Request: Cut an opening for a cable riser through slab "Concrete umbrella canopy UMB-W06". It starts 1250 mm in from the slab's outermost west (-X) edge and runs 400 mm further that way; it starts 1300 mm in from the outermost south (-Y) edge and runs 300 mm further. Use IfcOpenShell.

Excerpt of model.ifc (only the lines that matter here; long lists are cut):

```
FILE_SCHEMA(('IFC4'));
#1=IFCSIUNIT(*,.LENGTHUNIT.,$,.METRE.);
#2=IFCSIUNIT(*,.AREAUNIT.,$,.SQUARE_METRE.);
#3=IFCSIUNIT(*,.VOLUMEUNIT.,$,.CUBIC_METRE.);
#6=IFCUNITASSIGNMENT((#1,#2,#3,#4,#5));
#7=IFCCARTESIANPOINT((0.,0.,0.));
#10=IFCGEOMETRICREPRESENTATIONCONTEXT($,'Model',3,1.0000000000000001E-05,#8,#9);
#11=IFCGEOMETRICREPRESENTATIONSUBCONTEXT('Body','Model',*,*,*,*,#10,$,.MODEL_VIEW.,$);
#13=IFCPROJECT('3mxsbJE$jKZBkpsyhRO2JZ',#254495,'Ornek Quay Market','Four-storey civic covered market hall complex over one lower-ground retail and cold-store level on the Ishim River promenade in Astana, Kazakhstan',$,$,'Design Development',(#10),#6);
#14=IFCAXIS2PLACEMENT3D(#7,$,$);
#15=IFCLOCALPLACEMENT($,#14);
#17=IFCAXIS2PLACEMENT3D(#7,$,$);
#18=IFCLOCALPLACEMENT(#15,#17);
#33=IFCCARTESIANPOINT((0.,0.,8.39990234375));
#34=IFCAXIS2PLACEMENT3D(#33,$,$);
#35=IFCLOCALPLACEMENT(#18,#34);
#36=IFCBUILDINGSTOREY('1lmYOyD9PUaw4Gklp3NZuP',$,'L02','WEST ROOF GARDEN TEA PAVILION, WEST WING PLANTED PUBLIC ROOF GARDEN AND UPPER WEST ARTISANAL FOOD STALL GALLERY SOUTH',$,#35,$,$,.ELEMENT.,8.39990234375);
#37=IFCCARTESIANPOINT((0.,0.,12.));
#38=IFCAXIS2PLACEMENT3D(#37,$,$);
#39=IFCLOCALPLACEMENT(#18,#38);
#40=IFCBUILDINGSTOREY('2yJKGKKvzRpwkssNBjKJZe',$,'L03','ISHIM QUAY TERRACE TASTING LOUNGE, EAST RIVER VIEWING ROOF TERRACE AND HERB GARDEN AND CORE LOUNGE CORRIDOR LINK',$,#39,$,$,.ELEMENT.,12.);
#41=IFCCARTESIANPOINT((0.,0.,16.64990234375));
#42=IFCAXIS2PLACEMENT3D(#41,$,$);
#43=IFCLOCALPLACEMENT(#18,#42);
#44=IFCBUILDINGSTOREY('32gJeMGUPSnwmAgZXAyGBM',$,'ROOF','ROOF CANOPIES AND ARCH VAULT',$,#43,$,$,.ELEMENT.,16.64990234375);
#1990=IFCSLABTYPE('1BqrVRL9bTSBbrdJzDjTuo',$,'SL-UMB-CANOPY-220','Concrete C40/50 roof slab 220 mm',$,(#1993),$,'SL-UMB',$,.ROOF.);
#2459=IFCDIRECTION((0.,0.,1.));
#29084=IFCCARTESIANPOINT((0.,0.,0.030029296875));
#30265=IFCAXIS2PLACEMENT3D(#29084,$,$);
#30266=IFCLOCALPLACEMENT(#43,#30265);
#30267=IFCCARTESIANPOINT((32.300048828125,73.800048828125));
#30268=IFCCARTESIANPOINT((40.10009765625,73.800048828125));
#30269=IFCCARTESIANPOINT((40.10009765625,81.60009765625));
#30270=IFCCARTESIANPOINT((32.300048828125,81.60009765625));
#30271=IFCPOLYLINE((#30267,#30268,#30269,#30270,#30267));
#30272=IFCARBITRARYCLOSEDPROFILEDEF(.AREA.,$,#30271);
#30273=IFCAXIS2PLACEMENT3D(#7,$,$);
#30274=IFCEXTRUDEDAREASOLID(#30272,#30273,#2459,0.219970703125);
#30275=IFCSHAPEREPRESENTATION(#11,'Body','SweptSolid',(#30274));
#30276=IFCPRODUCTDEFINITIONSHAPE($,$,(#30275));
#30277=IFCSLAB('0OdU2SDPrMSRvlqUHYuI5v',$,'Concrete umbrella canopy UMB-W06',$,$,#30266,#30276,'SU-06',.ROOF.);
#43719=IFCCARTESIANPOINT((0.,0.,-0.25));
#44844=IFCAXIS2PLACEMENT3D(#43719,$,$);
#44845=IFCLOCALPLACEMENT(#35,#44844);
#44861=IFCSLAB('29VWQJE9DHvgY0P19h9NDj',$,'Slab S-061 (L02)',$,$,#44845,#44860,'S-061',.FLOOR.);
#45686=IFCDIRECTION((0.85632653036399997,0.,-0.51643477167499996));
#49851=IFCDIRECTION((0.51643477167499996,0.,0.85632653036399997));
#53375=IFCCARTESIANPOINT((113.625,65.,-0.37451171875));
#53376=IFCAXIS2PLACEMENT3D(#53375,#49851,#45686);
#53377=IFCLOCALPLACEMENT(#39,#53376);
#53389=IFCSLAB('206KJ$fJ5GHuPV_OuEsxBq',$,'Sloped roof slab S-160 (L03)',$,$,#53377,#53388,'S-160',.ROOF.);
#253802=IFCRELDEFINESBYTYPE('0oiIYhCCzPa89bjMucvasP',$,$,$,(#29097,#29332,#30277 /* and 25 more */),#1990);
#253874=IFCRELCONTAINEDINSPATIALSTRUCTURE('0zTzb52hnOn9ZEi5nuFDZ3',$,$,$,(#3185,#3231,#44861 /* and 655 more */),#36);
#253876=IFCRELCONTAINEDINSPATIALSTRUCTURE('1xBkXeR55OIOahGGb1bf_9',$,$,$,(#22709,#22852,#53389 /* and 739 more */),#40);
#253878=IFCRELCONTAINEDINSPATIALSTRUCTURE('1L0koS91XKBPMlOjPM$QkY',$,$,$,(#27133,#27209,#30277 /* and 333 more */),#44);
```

```python
import numpy as np
import ifcopenshell
import ifcopenshell.api.feature
import ifcopenshell.api.geometry
import ifcopenshell.api.root
import ifcopenshell.geom
import ifcopenshell.util.placement
import ifcopenshell.util.representation
import ifcopenshell.util.shape
import ifcopenshell.util.unit

model = ifcopenshell.open("model.ifc")
unit_scale = ifcopenshell.util.unit.calculate_unit_scale(model)
settings = ifcopenshell.geom.settings()


def volume(element):
    """Net volume in cubic metres, openings subtracted."""
    shape = ifcopenshell.geom.create_shape(settings, element)
    return ifcopenshell.util.shape.get_volume(shape.geometry)


slab = model.by_guid("0OdU2SDPrMSRvlqUHYuI5v")
before = volume(slab)

# Extent in the slab's own axes, in metres. The edges named are its -X and -Y sides.
slab_shape = ifcopenshell.geom.create_shape(settings, slab)
vertices = ifcopenshell.util.shape.get_vertices(slab_shape.geometry)
x_min, y_min, bottom = vertices.min(axis=0)
top = vertices[:, 2].max()

opening = ifcopenshell.api.root.create_entity(model, ifc_class="IfcOpeningElement", name="Cable riser opening", predefined_type="OPENING")
context = ifcopenshell.util.representation.get_context(model, "Model", "Body", "MODEL_VIEW")
width, depth = 0.4, 0.3
outline = [(0.0, 0.0), (width, 0.0), (width, depth), (0.0, depth), (0.0, 0.0)]
# Overshoot both faces by 50 mm so the cut is clean.
shape = ifcopenshell.api.geometry.add_slab_representation(
    model, context=context, depth=top - bottom + 0.1, polyline=outline
)
ifcopenshell.api.geometry.assign_representation(model, product=opening, representation=shape)

matrix = ifcopenshell.util.placement.get_local_placement(slab.ObjectPlacement)
matrix[:, 3] = matrix @ np.append(np.array([x_min + 1.25, y_min + 1.3, bottom - 0.05]) / unit_scale, 1.0)
ifcopenshell.api.geometry.edit_object_placement(model, product=opening, matrix=matrix, is_si=False)
ifcopenshell.api.feature.add_feature(model, feature=opening, element=slab)

after = volume(slab)

print(f"slab volume {before:.3f} -> {after:.3f} m3")

model.write("model_rev.ifc")
```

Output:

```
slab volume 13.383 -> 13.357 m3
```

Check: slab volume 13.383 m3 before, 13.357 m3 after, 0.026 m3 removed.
